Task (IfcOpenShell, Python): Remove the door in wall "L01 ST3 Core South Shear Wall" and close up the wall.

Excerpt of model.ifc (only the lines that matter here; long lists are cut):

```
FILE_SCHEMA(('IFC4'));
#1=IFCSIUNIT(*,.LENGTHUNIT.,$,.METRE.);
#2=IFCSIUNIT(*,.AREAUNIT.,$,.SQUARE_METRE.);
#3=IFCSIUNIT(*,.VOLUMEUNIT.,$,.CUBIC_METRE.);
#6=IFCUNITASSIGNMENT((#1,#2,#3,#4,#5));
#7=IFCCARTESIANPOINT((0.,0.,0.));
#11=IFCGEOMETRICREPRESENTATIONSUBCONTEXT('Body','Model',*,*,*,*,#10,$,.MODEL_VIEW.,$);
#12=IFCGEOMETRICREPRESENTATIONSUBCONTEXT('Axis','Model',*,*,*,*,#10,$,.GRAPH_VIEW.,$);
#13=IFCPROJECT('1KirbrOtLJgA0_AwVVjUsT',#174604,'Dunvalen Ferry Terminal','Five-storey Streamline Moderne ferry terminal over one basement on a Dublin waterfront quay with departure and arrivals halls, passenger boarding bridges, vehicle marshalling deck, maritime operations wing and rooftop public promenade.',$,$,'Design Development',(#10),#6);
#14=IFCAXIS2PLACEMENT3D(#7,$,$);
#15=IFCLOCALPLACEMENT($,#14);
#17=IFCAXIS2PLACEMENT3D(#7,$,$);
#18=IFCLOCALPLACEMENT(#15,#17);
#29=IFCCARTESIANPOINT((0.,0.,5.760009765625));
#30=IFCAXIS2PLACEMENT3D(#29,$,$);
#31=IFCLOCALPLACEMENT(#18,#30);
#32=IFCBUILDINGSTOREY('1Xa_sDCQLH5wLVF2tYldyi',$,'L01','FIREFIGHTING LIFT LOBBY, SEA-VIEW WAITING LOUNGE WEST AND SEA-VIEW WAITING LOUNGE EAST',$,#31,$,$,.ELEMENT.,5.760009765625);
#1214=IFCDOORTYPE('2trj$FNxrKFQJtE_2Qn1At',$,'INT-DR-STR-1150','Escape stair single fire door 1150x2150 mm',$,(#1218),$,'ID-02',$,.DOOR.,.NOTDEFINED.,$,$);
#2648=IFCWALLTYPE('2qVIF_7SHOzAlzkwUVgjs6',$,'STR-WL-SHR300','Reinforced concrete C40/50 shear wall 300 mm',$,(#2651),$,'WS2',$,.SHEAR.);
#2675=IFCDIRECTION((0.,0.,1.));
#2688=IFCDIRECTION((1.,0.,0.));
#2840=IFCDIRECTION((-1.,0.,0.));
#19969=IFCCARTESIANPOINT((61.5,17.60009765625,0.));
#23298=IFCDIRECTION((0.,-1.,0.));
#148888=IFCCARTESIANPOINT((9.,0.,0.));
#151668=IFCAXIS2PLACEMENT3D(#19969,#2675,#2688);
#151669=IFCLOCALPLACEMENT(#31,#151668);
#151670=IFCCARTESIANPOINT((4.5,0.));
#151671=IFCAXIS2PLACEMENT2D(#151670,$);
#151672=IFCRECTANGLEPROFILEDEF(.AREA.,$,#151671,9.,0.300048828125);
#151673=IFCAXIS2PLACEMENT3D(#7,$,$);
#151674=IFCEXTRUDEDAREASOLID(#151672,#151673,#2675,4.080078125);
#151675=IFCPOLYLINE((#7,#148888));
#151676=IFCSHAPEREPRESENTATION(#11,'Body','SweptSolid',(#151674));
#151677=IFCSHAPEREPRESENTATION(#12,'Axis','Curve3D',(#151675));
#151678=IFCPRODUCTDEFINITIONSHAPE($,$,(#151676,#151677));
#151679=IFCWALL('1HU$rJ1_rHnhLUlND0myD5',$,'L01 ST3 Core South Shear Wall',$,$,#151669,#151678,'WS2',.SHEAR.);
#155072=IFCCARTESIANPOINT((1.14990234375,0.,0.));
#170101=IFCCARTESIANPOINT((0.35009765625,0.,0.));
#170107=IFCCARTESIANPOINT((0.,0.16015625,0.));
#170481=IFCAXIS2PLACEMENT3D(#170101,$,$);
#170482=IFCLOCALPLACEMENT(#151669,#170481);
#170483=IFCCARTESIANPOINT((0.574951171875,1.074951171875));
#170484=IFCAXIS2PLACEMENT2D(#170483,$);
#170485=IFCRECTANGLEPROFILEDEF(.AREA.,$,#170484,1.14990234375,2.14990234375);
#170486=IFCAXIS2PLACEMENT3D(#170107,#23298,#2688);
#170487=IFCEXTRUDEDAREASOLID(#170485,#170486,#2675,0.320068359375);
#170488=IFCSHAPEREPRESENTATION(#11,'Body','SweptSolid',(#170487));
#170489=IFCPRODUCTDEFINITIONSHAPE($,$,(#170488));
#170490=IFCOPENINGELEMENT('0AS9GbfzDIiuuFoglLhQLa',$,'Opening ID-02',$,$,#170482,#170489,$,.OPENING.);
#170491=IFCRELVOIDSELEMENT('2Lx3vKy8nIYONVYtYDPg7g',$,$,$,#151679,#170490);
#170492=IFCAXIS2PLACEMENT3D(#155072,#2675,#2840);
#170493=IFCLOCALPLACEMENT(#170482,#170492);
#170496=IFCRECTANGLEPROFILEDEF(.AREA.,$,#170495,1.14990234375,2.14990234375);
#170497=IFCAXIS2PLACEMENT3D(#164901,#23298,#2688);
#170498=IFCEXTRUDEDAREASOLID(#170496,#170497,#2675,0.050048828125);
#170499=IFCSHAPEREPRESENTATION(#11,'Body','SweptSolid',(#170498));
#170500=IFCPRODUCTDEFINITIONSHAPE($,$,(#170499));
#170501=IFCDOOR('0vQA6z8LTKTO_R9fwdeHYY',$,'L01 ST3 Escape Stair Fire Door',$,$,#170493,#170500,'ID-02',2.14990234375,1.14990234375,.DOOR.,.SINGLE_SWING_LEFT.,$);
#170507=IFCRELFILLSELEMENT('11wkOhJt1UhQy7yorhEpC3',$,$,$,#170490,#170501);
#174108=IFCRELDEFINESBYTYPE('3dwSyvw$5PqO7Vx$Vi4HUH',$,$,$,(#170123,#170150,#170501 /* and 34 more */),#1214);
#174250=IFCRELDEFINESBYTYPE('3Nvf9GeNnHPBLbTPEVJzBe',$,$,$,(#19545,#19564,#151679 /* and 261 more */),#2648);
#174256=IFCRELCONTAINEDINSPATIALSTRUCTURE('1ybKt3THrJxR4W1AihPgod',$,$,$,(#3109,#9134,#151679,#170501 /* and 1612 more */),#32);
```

```python
import ifcopenshell
import ifcopenshell.api.feature
import ifcopenshell.api.root
import ifcopenshell.geom
import ifcopenshell.util.shape

model = ifcopenshell.open("model.ifc")
settings = ifcopenshell.geom.settings()


def volume(element):
    """Net volume in cubic metres, openings subtracted."""
    shape = ifcopenshell.geom.create_shape(settings, element)
    return ifcopenshell.util.shape.get_volume(shape.geometry)


door = model.by_id(170501)
opening = door.FillsVoids[0].RelatingOpeningElement
wall = opening.VoidsElements[0].RelatingBuildingElement
before = volume(wall)

ifcopenshell.api.root.remove_product(model, product=door)
ifcopenshell.api.feature.remove_feature(model, feature=opening)

after = volume(wall)

print(f"wall volume {before:.3f} -> {after:.3f} m3")

model.write("model_v2.ifc")
```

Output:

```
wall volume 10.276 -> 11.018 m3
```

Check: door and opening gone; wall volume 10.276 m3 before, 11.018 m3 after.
